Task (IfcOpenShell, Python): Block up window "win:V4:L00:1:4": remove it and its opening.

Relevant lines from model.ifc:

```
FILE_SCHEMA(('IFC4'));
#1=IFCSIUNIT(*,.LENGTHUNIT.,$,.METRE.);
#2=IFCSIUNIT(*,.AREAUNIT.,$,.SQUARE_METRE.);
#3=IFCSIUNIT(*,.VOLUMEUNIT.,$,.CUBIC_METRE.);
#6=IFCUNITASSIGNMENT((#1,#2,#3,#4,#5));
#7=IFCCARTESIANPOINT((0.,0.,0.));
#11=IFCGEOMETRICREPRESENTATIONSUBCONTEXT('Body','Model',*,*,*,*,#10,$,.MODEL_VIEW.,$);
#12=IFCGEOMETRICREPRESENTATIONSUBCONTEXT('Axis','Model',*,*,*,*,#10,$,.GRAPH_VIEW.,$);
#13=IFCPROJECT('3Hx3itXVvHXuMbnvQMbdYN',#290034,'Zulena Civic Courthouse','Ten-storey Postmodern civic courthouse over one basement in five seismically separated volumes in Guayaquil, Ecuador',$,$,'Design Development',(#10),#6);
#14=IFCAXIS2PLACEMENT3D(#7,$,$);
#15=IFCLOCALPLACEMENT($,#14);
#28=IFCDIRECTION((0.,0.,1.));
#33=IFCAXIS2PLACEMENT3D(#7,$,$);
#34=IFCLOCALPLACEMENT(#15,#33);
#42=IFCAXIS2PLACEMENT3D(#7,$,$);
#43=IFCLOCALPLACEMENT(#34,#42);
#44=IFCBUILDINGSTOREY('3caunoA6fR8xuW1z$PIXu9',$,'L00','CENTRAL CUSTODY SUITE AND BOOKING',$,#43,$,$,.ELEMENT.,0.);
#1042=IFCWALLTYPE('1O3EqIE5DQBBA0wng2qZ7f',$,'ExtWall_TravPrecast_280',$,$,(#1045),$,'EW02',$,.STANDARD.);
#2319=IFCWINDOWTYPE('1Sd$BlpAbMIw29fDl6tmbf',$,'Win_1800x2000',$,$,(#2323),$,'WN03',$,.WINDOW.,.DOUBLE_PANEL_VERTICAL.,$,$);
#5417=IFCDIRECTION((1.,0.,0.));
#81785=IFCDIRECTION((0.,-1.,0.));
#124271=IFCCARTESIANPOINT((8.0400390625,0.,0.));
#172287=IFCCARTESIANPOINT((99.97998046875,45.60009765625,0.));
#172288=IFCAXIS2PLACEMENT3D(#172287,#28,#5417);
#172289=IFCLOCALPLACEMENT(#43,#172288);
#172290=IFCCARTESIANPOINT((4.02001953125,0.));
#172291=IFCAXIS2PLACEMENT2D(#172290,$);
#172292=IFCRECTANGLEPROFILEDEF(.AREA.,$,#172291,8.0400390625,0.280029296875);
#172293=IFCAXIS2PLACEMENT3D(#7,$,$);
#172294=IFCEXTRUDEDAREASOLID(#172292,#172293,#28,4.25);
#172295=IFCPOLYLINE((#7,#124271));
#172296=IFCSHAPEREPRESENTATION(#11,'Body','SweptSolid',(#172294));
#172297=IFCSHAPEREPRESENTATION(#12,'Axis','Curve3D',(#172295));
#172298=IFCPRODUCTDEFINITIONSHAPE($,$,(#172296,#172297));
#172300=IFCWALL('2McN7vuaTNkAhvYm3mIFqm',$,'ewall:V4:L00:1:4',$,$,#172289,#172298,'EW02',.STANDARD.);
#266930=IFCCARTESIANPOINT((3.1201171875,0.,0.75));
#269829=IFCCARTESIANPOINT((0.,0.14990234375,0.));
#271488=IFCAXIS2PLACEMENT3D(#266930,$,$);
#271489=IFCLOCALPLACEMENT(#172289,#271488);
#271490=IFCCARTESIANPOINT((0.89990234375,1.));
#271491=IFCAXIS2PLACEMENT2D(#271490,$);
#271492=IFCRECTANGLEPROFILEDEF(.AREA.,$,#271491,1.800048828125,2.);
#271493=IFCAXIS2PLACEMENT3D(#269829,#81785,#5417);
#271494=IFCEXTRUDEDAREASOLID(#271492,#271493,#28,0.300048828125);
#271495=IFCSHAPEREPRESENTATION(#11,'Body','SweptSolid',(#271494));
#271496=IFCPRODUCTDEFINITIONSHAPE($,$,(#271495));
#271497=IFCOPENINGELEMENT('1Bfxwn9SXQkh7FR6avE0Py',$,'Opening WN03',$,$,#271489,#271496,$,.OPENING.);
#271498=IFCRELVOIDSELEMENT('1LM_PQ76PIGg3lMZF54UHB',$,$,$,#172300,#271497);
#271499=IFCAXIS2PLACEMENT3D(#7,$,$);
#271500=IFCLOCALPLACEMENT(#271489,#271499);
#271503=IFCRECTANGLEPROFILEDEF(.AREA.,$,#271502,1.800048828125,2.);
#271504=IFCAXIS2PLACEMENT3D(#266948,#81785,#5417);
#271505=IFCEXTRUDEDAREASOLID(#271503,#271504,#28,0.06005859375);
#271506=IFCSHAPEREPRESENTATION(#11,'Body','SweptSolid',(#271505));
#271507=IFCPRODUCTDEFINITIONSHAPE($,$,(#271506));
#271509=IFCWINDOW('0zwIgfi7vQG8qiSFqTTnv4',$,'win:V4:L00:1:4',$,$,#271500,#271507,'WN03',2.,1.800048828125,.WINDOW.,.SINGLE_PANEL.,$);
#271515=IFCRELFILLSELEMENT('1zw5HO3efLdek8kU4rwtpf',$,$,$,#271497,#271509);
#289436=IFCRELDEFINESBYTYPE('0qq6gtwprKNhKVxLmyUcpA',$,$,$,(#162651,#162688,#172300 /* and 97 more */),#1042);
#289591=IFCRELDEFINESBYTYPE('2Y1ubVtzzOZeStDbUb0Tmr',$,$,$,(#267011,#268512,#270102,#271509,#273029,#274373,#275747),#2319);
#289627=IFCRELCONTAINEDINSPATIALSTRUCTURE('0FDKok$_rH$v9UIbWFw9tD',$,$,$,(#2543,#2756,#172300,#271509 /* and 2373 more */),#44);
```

```python
import ifcopenshell
import ifcopenshell.api.feature
import ifcopenshell.api.root
import ifcopenshell.geom
import ifcopenshell.util.shape

model = ifcopenshell.open("model.ifc")
settings = ifcopenshell.geom.settings()


def volume(element):
    """Net volume in cubic metres, openings subtracted."""
    shape = ifcopenshell.geom.create_shape(settings, element)
    return ifcopenshell.util.shape.get_volume(shape.geometry)


window = model.by_id(271509)
opening = window.FillsVoids[0].RelatingOpeningElement
wall = opening.VoidsElements[0].RelatingBuildingElement
before = volume(wall)

ifcopenshell.api.root.remove_product(model, product=window)
ifcopenshell.api.feature.remove_feature(model, feature=opening)

after = volume(wall)

print(f"wall volume {before:.3f} -> {after:.3f} m3")

model.write("model-out.ifc")
```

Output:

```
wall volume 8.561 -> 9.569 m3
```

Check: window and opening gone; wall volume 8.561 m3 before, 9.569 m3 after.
